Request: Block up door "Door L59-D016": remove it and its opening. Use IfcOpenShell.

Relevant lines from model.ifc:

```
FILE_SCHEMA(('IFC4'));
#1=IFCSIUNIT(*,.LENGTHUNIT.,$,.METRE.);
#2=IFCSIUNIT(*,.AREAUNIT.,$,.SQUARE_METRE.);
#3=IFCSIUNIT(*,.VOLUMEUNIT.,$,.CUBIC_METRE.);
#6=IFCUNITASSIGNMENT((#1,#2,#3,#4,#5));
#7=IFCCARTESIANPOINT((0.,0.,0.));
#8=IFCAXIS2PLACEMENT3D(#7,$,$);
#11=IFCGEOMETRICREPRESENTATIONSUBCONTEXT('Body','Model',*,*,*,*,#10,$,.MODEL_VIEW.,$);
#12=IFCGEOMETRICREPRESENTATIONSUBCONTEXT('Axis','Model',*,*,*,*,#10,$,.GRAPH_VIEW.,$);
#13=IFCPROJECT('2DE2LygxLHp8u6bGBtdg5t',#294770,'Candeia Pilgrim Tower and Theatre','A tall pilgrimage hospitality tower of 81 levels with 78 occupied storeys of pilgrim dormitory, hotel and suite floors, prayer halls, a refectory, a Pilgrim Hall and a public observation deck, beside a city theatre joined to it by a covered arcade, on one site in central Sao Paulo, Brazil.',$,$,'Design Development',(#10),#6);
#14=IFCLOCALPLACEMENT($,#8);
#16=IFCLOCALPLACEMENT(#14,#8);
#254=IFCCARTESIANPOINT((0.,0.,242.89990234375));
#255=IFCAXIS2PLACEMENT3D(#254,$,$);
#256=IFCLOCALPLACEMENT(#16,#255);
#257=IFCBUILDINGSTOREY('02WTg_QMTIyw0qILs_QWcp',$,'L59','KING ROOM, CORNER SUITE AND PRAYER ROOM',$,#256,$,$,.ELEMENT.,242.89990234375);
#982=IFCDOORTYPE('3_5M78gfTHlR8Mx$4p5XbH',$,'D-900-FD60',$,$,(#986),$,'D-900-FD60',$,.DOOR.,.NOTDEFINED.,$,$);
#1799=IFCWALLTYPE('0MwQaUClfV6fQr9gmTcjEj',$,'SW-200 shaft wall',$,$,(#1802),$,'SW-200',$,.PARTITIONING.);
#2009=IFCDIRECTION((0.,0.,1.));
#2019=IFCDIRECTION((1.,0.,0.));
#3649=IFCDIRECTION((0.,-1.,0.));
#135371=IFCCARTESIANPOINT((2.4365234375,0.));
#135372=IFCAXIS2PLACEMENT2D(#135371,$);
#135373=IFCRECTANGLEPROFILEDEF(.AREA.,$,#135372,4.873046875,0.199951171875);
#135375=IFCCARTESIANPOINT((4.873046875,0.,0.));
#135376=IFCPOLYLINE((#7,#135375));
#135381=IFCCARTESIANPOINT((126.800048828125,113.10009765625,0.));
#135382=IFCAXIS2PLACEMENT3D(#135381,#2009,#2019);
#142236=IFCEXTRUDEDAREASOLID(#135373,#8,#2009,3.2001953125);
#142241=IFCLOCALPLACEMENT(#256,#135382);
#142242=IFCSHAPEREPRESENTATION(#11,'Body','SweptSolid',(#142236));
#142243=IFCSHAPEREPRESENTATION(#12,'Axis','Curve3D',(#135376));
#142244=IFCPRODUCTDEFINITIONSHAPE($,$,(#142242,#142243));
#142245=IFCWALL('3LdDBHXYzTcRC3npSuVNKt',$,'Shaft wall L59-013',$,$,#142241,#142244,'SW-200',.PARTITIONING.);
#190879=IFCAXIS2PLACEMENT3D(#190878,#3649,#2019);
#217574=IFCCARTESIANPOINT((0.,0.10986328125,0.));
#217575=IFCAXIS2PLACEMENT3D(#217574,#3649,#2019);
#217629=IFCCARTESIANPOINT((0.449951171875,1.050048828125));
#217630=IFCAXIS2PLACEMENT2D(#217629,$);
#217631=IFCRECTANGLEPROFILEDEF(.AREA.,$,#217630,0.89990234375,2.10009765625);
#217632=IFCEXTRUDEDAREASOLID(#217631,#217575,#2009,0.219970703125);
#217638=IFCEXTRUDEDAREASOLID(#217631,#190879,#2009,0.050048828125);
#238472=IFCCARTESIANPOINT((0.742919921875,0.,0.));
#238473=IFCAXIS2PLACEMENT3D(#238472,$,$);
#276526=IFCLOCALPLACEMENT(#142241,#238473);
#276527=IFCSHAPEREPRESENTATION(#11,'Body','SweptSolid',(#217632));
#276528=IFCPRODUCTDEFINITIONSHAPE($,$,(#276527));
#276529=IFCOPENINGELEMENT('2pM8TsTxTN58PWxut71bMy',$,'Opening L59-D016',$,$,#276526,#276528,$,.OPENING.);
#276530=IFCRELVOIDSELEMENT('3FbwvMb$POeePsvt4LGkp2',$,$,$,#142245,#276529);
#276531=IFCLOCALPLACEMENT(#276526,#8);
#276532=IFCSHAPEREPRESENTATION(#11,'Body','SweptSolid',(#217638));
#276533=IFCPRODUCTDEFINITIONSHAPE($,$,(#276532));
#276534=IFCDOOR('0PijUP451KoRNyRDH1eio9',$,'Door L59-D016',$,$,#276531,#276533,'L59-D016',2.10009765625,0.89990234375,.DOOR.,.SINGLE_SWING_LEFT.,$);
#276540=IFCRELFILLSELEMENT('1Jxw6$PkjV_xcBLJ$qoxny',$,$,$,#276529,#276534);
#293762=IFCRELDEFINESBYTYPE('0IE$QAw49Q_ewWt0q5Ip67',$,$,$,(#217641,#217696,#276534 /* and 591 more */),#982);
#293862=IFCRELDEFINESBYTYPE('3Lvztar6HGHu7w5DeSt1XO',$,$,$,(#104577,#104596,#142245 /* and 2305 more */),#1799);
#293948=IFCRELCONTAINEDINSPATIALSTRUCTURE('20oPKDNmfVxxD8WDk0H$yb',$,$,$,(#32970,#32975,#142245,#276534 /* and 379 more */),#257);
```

```python
import ifcopenshell
import ifcopenshell.api.feature
import ifcopenshell.api.root
import ifcopenshell.geom
import ifcopenshell.util.shape

model = ifcopenshell.open("model.ifc")
settings = ifcopenshell.geom.settings()


def volume(element):
    """Net volume in cubic metres, openings subtracted."""
    shape = ifcopenshell.geom.create_shape(settings, element)
    return ifcopenshell.util.shape.get_volume(shape.geometry)


door = model.by_guid("0PijUP451KoRNyRDH1eio9")
opening = door.FillsVoids[0].RelatingOpeningElement
wall = opening.VoidsElements[0].RelatingBuildingElement
before = volume(wall)

ifcopenshell.api.root.remove_product(model, product=door)
ifcopenshell.api.feature.remove_feature(model, feature=opening)

after = volume(wall)

print(f"wall volume {before:.3f} -> {after:.3f} m3")

model.write("model-out.ifc")
```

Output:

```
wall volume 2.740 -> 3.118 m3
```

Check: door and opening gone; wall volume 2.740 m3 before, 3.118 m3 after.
